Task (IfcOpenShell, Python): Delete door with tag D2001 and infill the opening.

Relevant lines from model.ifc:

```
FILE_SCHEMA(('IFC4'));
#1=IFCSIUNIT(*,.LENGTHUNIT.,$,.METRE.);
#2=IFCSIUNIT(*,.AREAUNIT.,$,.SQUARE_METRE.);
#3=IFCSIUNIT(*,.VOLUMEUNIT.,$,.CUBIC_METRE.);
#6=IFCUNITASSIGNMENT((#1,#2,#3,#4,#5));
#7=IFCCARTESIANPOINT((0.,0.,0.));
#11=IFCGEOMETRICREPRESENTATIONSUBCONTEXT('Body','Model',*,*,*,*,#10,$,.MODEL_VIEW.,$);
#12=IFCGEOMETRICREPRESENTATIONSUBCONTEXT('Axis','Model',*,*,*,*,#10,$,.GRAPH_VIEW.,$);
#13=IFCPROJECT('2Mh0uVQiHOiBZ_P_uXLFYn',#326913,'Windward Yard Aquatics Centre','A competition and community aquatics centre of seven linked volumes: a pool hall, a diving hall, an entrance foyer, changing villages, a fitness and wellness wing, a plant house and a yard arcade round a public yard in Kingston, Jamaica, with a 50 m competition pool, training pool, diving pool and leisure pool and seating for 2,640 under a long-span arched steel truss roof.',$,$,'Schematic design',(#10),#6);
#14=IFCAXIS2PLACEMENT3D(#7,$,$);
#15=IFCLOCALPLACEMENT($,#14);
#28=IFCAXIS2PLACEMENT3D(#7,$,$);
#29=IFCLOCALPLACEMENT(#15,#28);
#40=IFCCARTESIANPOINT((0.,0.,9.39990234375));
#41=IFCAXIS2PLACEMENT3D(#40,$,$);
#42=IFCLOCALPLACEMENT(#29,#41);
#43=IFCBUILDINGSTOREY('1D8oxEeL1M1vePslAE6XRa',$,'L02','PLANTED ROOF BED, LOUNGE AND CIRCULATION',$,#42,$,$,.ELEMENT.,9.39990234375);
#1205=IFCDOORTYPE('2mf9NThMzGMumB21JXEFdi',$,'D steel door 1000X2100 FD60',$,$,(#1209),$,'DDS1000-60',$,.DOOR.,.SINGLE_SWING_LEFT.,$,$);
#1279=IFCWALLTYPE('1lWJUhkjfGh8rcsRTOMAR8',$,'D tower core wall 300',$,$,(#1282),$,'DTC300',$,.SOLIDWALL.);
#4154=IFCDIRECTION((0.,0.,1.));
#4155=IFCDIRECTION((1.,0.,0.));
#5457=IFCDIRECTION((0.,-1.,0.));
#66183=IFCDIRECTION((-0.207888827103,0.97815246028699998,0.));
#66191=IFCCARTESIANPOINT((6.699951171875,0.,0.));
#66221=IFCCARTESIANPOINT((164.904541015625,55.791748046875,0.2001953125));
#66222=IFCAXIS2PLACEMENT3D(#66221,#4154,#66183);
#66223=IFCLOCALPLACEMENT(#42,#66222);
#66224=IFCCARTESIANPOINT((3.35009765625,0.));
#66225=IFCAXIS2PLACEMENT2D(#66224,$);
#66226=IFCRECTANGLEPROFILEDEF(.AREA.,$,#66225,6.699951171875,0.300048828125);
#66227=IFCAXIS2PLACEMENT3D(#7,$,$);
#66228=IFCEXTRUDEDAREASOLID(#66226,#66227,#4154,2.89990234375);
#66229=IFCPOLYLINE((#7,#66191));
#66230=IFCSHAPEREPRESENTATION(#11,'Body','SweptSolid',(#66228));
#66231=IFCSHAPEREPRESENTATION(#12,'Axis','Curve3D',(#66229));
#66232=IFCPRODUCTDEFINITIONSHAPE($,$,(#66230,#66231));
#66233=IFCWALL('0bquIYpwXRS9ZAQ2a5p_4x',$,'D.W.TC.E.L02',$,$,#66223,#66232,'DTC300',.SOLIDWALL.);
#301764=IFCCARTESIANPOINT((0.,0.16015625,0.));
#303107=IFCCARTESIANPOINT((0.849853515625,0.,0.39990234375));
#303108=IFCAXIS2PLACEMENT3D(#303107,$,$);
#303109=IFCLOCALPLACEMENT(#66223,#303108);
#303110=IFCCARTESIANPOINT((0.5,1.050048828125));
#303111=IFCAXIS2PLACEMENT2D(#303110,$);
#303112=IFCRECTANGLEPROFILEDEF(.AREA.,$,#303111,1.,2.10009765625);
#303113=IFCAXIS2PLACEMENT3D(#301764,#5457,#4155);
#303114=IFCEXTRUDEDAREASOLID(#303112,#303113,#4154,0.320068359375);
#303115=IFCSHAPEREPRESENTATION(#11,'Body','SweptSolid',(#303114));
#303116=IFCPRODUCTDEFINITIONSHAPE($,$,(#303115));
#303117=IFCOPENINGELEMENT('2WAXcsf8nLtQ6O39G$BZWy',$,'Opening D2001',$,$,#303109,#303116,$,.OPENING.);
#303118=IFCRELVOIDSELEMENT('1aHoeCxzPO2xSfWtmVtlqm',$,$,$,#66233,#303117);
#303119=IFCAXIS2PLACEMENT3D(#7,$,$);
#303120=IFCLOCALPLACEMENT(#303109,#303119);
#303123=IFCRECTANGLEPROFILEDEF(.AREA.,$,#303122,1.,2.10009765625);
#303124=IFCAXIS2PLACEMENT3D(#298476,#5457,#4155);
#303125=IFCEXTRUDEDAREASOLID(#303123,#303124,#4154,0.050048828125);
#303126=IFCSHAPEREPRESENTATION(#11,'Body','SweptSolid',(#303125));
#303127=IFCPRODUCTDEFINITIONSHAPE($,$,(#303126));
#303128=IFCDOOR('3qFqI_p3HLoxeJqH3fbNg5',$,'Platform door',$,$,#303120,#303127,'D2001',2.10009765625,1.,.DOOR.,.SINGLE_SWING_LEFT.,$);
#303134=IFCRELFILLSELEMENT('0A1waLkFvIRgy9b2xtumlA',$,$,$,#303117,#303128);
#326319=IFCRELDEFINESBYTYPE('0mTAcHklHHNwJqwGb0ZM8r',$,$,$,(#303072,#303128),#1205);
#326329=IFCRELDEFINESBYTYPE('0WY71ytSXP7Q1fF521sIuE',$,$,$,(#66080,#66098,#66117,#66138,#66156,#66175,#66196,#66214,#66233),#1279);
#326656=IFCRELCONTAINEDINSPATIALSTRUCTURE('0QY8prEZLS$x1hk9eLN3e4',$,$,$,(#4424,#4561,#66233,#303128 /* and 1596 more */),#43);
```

```python
import ifcopenshell
import ifcopenshell.api.feature
import ifcopenshell.api.root
import ifcopenshell.geom
import ifcopenshell.util.shape

model = ifcopenshell.open("model.ifc")
settings = ifcopenshell.geom.settings()


def volume(element):
    """Net volume in cubic metres, openings subtracted."""
    shape = ifcopenshell.geom.create_shape(settings, element)
    return ifcopenshell.util.shape.get_volume(shape.geometry)


door = model.by_guid("3qFqI_p3HLoxeJqH3fbNg5")
opening = door.FillsVoids[0].RelatingOpeningElement
wall = opening.VoidsElements[0].RelatingBuildingElement
before = volume(wall)

ifcopenshell.api.root.remove_product(model, product=door)
ifcopenshell.api.feature.remove_feature(model, feature=opening)

after = volume(wall)

print(f"wall volume {before:.3f} -> {after:.3f} m3")

model.write("model_v2.ifc")
```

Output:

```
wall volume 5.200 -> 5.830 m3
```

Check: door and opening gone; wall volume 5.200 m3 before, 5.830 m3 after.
